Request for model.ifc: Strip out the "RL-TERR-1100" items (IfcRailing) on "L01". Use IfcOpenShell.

First a look at what the model holds.

```python
import ifcopenshell
import ifcopenshell.util.element

model = ifcopenshell.open("model.ifc")
print(model.schema)
storey = next(s for s in model.by_type("IfcBuildingStorey") if s.Name == "L01")
railings = [e for e in ifcopenshell.util.element.get_decomposition(storey) if e.is_a("IfcRailing")]
seen = {}
for e in railings:
    element_type = ifcopenshell.util.element.get_type(e)
    name = element_type.Name if element_type not in (None, e) else None
    seen[name] = seen.get(name, 0) + 1
for name, count in sorted(seen.items(), key=str):
    print(count, "x", name)
```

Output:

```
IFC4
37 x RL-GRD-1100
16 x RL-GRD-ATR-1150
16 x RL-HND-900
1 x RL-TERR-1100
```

```python
import ifcopenshell
import ifcopenshell.api.root
import ifcopenshell.util.element

model = ifcopenshell.open("model.ifc")

storey = next(s for s in model.by_type("IfcBuildingStorey") if s.Name == "L01")
railings = [e for e in ifcopenshell.util.element.get_decomposition(storey) if e.is_a("IfcRailing")]
targets = [e for e in railings if (t := ifcopenshell.util.element.get_type(e)) not in (None, e) and t.Name == "RL-TERR-1100"]

for e in targets:
    ifcopenshell.api.root.remove_product(model, product=e)
print(len(targets), "removed")

model.write("model-out.ifc")
```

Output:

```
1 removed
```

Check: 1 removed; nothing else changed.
